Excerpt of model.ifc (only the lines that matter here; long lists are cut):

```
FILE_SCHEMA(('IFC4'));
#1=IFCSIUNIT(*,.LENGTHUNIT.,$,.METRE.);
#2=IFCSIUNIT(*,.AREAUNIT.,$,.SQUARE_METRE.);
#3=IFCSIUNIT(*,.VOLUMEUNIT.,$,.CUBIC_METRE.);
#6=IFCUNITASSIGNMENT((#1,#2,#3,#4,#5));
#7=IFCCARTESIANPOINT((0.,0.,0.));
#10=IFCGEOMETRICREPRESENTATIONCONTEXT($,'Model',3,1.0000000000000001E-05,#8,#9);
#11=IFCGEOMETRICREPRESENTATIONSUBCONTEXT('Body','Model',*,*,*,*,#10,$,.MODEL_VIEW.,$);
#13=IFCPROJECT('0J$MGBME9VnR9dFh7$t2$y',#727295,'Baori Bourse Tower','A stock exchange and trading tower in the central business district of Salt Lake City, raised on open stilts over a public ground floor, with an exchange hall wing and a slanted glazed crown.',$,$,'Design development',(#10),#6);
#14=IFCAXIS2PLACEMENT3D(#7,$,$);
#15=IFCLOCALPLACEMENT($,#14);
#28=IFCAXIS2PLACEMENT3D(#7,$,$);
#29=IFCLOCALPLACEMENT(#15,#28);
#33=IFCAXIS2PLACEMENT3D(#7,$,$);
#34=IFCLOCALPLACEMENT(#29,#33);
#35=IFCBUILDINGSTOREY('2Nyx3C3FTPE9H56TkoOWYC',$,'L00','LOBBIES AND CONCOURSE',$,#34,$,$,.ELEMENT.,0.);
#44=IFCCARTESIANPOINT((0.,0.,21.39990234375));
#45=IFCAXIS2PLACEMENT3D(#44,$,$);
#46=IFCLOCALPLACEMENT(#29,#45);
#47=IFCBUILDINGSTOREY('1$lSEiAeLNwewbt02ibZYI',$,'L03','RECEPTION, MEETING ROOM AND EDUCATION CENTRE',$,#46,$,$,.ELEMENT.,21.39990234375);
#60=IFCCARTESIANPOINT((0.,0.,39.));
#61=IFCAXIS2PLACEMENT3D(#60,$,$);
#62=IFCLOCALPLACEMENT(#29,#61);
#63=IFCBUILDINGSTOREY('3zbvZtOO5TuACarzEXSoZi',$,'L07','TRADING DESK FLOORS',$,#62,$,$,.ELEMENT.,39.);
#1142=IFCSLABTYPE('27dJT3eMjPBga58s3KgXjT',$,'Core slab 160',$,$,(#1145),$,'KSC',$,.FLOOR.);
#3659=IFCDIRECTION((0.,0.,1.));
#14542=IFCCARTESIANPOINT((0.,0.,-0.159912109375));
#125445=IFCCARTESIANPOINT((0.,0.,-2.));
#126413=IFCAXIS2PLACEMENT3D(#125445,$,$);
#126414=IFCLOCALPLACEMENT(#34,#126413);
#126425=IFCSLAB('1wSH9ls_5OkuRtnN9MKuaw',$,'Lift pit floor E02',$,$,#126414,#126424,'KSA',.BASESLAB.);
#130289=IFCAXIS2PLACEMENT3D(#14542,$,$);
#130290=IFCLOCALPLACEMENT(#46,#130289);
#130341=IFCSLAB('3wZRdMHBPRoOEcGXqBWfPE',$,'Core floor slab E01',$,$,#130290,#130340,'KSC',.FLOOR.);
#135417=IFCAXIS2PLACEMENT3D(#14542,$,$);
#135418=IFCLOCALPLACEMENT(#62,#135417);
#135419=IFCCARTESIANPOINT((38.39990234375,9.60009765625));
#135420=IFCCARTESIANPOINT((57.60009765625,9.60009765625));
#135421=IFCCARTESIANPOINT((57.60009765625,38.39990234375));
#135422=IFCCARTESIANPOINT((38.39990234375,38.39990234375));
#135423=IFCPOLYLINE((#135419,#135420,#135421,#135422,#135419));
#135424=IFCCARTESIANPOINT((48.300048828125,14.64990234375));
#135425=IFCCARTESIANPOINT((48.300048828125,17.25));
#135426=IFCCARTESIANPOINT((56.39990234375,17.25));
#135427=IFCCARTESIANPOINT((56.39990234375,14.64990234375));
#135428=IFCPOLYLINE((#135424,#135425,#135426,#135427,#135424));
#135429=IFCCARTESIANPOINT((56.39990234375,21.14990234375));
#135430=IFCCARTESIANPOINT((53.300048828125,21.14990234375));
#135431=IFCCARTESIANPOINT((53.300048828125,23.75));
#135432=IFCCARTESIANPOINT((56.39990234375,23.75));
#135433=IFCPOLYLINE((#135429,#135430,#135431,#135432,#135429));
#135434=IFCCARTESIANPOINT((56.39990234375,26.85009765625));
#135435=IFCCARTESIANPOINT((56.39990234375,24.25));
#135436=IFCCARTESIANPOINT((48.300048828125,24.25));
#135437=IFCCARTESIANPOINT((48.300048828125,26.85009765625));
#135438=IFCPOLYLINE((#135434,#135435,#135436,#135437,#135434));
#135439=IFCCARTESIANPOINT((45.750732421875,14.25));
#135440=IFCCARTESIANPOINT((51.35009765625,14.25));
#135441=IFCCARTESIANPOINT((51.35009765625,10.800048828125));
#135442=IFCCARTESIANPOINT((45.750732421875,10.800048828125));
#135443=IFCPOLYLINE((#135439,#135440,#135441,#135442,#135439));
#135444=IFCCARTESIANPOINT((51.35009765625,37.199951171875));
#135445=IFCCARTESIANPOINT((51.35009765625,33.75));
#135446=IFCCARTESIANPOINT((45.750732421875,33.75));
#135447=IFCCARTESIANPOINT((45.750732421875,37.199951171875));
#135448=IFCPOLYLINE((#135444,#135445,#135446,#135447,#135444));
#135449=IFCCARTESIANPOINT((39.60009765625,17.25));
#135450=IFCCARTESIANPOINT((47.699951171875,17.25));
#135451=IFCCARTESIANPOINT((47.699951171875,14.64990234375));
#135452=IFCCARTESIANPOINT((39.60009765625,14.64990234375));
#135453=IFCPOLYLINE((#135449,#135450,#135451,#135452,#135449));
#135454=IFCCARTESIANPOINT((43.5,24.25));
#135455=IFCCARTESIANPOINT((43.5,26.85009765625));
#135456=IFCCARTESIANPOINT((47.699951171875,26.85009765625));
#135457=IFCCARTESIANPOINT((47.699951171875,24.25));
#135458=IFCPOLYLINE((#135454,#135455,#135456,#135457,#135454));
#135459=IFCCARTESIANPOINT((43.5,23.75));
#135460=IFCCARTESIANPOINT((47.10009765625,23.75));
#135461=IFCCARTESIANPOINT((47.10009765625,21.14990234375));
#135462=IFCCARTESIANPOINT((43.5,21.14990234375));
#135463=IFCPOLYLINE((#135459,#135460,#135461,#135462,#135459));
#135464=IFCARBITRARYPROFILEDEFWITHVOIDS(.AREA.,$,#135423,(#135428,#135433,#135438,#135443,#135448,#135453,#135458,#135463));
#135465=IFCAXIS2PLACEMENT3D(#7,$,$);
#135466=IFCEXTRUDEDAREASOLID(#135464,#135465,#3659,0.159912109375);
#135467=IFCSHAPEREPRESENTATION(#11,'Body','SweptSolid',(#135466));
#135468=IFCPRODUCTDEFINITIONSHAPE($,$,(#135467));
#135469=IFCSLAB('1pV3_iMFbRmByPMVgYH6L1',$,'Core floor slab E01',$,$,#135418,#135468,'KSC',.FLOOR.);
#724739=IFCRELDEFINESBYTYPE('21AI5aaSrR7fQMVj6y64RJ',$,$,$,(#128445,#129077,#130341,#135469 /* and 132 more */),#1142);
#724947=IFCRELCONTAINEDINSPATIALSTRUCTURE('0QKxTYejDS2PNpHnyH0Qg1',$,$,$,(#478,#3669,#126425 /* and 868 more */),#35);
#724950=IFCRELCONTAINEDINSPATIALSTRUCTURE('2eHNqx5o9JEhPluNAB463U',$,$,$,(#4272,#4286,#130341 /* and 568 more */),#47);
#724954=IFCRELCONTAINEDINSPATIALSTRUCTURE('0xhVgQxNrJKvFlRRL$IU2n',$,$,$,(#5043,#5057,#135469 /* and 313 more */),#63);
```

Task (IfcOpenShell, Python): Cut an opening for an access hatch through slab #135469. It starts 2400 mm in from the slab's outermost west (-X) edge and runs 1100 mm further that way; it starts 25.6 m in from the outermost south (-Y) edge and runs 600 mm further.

```python
import numpy as np
import ifcopenshell
import ifcopenshell.api.feature
import ifcopenshell.api.geometry
import ifcopenshell.api.root
import ifcopenshell.geom
import ifcopenshell.util.placement
import ifcopenshell.util.representation
import ifcopenshell.util.shape
import ifcopenshell.util.unit

model = ifcopenshell.open("model.ifc")
unit_scale = ifcopenshell.util.unit.calculate_unit_scale(model)
settings = ifcopenshell.geom.settings()


def volume(element):
    """Net volume in cubic metres, openings subtracted."""
    shape = ifcopenshell.geom.create_shape(settings, element)
    return ifcopenshell.util.shape.get_volume(shape.geometry)


slab = model.by_guid("1pV3_iMFbRmByPMVgYH6L1")
before = volume(slab)

# Extent in the slab's own axes, in metres. The edges named are its -X and -Y sides.
slab_shape = ifcopenshell.geom.create_shape(settings, slab)
vertices = ifcopenshell.util.shape.get_vertices(slab_shape.geometry)
x_min, y_min, bottom = vertices.min(axis=0)
top = vertices[:, 2].max()

opening = ifcopenshell.api.root.create_entity(model, ifc_class="IfcOpeningElement", name="Access hatch opening", predefined_type="OPENING")
context = ifcopenshell.util.representation.get_context(model, "Model", "Body", "MODEL_VIEW")
width, depth = 1.1, 0.6
outline = [(0.0, 0.0), (width, 0.0), (width, depth), (0.0, depth), (0.0, 0.0)]
# Overshoot both faces by 50 mm so the cut is clean.
shape = ifcopenshell.api.geometry.add_slab_representation(
    model, context=context, depth=top - bottom + 0.1, polyline=outline
)
ifcopenshell.api.geometry.assign_representation(model, product=opening, representation=shape)

matrix = ifcopenshell.util.placement.get_local_placement(slab.ObjectPlacement)
matrix[:, 3] = matrix @ np.append(np.array([x_min + 2.4, y_min + 25.6, bottom - 0.05]) / unit_scale, 1.0)
ifcopenshell.api.geometry.edit_object_placement(model, product=opening, matrix=matrix, is_si=False)
ifcopenshell.api.feature.add_feature(model, feature=opening, element=slab)

after = volume(slab)

print(f"slab volume {before:.3f} -> {after:.3f} m3")

model.write("model_v2.ifc")
```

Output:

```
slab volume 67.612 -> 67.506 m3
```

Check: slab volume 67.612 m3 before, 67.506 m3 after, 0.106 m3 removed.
